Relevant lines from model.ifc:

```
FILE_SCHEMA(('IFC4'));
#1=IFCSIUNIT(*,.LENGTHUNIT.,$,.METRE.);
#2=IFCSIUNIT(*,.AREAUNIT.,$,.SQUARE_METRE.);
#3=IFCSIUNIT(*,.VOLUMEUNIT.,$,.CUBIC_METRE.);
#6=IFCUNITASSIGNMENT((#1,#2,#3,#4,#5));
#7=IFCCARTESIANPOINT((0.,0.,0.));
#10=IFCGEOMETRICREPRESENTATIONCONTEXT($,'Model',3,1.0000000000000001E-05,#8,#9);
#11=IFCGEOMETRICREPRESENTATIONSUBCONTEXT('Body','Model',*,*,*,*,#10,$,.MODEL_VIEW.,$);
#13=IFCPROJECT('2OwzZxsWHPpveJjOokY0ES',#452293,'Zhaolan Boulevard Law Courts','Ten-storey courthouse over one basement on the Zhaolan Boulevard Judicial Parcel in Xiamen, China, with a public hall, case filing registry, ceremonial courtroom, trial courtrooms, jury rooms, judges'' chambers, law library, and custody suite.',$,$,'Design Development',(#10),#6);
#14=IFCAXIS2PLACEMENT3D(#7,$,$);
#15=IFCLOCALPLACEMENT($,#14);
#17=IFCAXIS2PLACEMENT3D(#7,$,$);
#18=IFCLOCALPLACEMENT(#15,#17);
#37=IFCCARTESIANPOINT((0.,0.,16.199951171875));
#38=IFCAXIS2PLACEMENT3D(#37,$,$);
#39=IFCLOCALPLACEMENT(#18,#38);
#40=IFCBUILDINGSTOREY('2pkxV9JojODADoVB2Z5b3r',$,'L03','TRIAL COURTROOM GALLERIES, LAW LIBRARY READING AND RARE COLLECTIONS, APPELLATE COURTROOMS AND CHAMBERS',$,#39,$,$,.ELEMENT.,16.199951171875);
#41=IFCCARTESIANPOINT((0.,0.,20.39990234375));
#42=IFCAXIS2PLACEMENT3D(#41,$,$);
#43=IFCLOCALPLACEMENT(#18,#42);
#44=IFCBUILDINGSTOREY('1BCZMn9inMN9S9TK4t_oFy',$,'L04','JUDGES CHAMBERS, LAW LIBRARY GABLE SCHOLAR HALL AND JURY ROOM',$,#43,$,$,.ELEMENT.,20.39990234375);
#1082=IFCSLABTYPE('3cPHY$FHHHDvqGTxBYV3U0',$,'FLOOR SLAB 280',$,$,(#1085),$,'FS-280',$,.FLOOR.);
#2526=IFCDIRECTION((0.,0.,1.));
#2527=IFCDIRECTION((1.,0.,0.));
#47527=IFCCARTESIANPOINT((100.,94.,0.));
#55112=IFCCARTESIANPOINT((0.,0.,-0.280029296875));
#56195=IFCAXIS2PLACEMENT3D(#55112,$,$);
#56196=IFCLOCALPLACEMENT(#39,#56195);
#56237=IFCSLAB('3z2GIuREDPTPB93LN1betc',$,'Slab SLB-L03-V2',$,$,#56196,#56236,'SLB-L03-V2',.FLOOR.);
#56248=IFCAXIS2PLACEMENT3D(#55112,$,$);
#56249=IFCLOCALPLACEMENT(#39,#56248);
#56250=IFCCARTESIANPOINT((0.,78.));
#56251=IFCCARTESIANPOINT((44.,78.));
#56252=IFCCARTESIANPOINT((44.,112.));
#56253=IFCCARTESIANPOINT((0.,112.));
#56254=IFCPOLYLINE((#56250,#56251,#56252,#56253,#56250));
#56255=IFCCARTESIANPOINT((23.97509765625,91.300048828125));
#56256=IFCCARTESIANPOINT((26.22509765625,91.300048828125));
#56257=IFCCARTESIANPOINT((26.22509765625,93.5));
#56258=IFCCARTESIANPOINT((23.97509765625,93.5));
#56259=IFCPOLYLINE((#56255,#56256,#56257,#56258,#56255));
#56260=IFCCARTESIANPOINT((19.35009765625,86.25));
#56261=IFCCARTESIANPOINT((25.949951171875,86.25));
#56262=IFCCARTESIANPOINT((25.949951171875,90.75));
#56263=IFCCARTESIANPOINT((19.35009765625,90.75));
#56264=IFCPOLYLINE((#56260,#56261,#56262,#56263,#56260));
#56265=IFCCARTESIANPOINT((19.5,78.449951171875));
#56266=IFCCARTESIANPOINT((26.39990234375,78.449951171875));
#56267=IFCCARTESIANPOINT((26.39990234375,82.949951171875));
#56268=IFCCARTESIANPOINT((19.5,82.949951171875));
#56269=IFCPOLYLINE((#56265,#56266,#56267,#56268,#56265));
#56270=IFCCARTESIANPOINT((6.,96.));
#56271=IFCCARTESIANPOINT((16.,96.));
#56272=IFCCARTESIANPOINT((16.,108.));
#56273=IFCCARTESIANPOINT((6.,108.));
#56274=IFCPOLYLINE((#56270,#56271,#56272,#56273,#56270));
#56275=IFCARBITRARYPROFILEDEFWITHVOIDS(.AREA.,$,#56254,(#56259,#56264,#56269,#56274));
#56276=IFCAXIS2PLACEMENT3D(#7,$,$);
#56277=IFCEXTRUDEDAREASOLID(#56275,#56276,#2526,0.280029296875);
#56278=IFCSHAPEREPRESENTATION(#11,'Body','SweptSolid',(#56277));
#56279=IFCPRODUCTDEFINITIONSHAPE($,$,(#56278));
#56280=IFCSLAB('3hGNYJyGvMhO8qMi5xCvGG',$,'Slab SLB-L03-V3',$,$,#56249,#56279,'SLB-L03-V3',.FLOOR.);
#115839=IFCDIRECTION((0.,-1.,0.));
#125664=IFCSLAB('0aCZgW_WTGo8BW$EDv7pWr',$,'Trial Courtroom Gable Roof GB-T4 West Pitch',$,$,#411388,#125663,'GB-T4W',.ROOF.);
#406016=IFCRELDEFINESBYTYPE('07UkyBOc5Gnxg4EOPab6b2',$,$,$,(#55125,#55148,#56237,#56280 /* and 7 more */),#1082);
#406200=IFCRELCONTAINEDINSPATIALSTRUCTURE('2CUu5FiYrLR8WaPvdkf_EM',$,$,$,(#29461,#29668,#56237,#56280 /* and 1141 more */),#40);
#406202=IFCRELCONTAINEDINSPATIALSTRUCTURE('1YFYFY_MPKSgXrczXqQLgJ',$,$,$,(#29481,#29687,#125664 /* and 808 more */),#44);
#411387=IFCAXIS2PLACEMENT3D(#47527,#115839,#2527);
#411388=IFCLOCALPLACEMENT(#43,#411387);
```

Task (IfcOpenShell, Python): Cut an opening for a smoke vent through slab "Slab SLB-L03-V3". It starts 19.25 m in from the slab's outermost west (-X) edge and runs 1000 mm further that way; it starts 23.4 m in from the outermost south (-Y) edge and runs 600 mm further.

```python
import numpy as np
import ifcopenshell
import ifcopenshell.api.feature
import ifcopenshell.api.geometry
import ifcopenshell.api.root
import ifcopenshell.geom
import ifcopenshell.util.placement
import ifcopenshell.util.representation
import ifcopenshell.util.shape
import ifcopenshell.util.unit

model = ifcopenshell.open("model.ifc")
unit_scale = ifcopenshell.util.unit.calculate_unit_scale(model)
settings = ifcopenshell.geom.settings()


def volume(element):
    """Net volume in cubic metres, openings subtracted."""
    shape = ifcopenshell.geom.create_shape(settings, element)
    return ifcopenshell.util.shape.get_volume(shape.geometry)


slab = model.by_guid("3hGNYJyGvMhO8qMi5xCvGG")
before = volume(slab)

# Extent in the slab's own axes, in metres. The edges named are its -X and -Y sides.
slab_shape = ifcopenshell.geom.create_shape(settings, slab)
vertices = ifcopenshell.util.shape.get_vertices(slab_shape.geometry)
x_min, y_min, bottom = vertices.min(axis=0)
top = vertices[:, 2].max()

opening = ifcopenshell.api.root.create_entity(model, ifc_class="IfcOpeningElement", name="Smoke vent opening", predefined_type="OPENING")
context = ifcopenshell.util.representation.get_context(model, "Model", "Body", "MODEL_VIEW")
width, depth = 1, 0.6
outline = [(0.0, 0.0), (width, 0.0), (width, depth), (0.0, depth), (0.0, 0.0)]
# Overshoot both faces by 50 mm so the cut is clean.
shape = ifcopenshell.api.geometry.add_slab_representation(
    model, context=context, depth=top - bottom + 0.1, polyline=outline
)
ifcopenshell.api.geometry.assign_representation(model, product=opening, representation=shape)

matrix = ifcopenshell.util.placement.get_local_placement(slab.ObjectPlacement)
matrix[:, 3] = matrix @ np.append(np.array([x_min + 19.25, y_min + 23.4, bottom - 0.05]) / unit_scale, 1.0)
ifcopenshell.api.geometry.edit_object_placement(model, product=opening, matrix=matrix, is_si=False)
ifcopenshell.api.feature.add_feature(model, feature=opening, element=slab)

after = volume(slab)

print(f"slab volume {before:.3f} -> {after:.3f} m3")

model.write("model-out.ifc")
```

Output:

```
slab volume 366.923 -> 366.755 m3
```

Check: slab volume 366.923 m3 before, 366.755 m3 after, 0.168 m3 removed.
